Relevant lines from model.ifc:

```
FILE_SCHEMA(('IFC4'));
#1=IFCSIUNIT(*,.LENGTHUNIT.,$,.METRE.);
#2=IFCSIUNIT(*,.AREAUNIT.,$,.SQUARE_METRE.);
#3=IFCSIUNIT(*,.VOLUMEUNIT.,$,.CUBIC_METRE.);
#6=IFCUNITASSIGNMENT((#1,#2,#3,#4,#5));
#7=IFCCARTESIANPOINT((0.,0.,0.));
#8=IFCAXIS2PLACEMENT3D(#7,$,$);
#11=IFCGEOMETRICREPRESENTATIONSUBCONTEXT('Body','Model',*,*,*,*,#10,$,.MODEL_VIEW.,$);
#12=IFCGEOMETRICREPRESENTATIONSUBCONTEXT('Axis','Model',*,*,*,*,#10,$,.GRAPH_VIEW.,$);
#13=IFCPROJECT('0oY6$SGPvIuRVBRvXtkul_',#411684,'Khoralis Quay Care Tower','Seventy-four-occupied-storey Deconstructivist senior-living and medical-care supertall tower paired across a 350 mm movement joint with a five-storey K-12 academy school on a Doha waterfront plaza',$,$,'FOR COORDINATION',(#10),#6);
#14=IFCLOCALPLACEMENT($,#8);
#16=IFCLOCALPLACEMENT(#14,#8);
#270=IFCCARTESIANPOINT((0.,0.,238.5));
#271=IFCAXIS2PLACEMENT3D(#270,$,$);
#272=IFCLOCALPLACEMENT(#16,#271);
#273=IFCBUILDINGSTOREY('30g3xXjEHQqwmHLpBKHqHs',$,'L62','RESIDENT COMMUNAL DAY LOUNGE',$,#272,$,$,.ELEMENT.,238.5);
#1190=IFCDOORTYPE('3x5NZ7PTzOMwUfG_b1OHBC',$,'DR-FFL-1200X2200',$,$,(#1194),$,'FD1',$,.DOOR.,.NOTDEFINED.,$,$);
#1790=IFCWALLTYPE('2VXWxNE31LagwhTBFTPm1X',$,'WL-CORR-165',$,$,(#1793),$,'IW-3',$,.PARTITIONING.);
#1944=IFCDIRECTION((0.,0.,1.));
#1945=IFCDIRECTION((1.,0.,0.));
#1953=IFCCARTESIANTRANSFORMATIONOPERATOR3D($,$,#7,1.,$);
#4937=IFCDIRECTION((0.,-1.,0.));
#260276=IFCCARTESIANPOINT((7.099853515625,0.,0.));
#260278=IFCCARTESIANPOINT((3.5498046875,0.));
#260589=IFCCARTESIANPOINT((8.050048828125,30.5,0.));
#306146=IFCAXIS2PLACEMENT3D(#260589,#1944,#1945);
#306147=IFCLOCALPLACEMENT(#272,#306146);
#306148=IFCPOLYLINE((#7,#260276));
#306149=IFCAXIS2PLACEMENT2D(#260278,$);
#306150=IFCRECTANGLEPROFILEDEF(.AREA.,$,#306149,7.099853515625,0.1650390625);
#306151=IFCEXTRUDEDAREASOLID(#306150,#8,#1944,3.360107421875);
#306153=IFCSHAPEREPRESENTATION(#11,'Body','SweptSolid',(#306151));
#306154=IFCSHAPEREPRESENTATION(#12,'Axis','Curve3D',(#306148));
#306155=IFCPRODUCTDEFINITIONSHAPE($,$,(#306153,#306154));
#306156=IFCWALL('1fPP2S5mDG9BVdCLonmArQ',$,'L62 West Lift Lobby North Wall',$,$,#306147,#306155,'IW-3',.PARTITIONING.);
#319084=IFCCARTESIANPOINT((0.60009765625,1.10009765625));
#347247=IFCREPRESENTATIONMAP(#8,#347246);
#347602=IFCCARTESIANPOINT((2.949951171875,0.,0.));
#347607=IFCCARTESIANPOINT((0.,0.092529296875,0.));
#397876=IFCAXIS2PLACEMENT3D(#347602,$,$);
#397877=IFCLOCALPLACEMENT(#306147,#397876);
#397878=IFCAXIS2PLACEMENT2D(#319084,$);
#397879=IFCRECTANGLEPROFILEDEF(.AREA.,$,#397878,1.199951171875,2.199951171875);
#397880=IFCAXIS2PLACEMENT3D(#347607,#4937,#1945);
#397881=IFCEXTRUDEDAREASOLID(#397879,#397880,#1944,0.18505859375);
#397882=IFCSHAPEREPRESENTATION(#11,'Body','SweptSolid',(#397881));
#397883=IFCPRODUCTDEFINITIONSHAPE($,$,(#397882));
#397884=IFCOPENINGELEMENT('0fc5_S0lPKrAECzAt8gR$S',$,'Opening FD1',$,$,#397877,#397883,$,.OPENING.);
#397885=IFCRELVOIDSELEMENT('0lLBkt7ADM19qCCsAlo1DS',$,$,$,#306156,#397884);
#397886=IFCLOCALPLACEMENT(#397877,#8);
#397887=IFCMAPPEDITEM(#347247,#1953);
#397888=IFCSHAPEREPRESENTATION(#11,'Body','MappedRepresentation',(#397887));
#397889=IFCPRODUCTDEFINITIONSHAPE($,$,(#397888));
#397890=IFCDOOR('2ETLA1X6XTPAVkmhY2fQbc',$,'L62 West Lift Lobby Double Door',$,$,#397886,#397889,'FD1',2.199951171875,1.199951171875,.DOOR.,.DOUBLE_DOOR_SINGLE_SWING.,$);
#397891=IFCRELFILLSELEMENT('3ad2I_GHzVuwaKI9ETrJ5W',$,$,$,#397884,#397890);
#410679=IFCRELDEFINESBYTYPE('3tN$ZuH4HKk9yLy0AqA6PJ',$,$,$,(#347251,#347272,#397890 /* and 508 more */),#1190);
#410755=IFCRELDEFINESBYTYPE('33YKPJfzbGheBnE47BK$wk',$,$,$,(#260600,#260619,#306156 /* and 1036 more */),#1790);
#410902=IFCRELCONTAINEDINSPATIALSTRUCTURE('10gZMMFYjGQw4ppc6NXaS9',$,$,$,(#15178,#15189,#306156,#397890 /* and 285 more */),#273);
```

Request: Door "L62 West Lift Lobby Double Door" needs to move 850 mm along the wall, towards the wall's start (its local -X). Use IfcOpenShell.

```python
import ifcopenshell
import ifcopenshell.api.geometry
import ifcopenshell.util.placement

model = ifcopenshell.open("model.ifc")

door = model.by_id(397890)
opening = door.FillsVoids[0].RelatingOpeningElement
wall = opening.VoidsElements[0].RelatingBuildingElement

wall_matrix = ifcopenshell.util.placement.get_local_placement(wall.ObjectPlacement)
shift = wall_matrix[:3, 0] * -0.85
before = ifcopenshell.util.placement.get_local_placement(door.ObjectPlacement)[:3, 3].copy()

# The door is placed relative to its opening, so it follows when the opening moves.
matrix = ifcopenshell.util.placement.get_local_placement(opening.ObjectPlacement)
matrix[:3, 3] += shift
ifcopenshell.api.geometry.edit_object_placement(
    model, product=opening, matrix=matrix, is_si=False, should_transform_children=True
)

after = ifcopenshell.util.placement.get_local_placement(door.ObjectPlacement)[:3, 3]
print("door moved by", (after - before).round(3) + 0.0)

model.write("model_v2.ifc")
```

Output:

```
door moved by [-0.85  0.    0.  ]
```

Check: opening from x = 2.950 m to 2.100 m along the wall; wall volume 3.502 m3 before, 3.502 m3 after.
